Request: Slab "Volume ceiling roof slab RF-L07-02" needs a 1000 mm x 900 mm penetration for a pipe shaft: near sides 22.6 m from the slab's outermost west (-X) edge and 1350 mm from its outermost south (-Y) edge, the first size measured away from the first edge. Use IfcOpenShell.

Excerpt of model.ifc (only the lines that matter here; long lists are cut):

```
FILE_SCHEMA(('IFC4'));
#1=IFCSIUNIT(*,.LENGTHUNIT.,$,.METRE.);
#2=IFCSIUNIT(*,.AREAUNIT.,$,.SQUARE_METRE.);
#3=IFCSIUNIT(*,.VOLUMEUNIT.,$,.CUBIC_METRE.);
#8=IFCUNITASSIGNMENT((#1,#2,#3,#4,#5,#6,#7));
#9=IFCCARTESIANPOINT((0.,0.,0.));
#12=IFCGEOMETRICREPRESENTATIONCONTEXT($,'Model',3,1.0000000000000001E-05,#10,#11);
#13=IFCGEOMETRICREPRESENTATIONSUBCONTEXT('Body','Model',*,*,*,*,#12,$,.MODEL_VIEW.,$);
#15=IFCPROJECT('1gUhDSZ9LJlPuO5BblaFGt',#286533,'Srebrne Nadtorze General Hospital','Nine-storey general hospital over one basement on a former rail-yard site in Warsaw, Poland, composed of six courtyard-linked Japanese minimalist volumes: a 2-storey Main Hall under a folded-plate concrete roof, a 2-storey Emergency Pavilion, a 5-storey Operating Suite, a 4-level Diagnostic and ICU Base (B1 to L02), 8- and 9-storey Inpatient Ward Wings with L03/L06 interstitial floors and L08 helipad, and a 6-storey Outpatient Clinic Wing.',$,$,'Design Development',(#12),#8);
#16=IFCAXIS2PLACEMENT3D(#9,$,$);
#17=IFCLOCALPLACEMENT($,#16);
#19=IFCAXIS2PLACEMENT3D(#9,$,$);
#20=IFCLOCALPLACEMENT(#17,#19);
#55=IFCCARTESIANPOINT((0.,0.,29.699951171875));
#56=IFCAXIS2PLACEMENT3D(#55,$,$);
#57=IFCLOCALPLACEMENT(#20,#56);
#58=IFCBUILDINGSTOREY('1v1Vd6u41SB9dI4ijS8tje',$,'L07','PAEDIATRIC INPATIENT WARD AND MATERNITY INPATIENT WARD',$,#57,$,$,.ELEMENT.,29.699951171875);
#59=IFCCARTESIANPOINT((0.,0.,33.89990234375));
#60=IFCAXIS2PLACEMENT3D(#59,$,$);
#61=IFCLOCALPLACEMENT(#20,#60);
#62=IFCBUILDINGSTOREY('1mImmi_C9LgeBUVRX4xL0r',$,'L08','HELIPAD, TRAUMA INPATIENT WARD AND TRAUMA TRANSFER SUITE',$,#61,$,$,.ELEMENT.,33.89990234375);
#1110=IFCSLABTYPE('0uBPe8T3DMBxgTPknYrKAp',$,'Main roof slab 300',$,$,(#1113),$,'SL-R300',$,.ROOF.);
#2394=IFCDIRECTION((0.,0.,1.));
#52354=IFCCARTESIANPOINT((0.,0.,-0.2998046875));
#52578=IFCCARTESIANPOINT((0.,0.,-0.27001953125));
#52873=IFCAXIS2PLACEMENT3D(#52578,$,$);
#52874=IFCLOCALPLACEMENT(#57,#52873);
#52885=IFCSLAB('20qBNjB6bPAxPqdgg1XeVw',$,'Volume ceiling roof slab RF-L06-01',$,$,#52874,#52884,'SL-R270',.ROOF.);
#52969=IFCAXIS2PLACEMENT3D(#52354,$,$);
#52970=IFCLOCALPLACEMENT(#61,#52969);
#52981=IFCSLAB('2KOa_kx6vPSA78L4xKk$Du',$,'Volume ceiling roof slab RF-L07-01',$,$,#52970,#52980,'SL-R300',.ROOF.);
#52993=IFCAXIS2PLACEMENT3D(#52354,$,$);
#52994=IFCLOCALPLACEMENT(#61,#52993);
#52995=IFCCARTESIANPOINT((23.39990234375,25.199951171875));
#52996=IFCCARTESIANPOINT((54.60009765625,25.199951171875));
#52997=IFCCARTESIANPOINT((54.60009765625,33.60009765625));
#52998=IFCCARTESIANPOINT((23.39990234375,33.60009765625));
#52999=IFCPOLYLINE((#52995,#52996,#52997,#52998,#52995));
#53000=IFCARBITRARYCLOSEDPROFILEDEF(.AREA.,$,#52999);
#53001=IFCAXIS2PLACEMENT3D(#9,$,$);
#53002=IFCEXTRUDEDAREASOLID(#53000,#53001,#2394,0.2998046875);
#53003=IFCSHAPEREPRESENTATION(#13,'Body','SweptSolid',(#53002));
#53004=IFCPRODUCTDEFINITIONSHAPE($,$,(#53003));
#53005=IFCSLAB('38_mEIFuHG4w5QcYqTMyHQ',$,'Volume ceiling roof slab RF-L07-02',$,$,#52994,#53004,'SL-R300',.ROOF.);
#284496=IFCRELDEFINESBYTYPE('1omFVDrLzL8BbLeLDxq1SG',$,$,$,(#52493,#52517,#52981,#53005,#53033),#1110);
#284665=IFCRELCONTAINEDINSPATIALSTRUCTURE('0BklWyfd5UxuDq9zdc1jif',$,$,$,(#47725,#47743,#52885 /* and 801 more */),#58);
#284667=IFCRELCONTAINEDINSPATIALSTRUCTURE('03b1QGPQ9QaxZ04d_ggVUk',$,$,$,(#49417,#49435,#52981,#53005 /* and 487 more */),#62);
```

```python
import numpy as np
import ifcopenshell
import ifcopenshell.api.feature
import ifcopenshell.api.geometry
import ifcopenshell.api.root
import ifcopenshell.geom
import ifcopenshell.util.placement
import ifcopenshell.util.representation
import ifcopenshell.util.shape
import ifcopenshell.util.unit

model = ifcopenshell.open("model.ifc")
unit_scale = ifcopenshell.util.unit.calculate_unit_scale(model)
settings = ifcopenshell.geom.settings()


def volume(element):
    """Net volume in cubic metres, openings subtracted."""
    shape = ifcopenshell.geom.create_shape(settings, element)
    return ifcopenshell.util.shape.get_volume(shape.geometry)


slab = model.by_guid("38_mEIFuHG4w5QcYqTMyHQ")
before = volume(slab)

# Extent in the slab's own axes, in metres. The edges named are its -X and -Y sides.
slab_shape = ifcopenshell.geom.create_shape(settings, slab)
vertices = ifcopenshell.util.shape.get_vertices(slab_shape.geometry)
x_min, y_min, bottom = vertices.min(axis=0)
top = vertices[:, 2].max()

opening = ifcopenshell.api.root.create_entity(model, ifc_class="IfcOpeningElement", name="Pipe shaft opening", predefined_type="OPENING")
context = ifcopenshell.util.representation.get_context(model, "Model", "Body", "MODEL_VIEW")
width, depth = 1, 0.9
outline = [(0.0, 0.0), (width, 0.0), (width, depth), (0.0, depth), (0.0, 0.0)]
# Overshoot both faces by 50 mm so the cut is clean.
shape = ifcopenshell.api.geometry.add_slab_representation(
    model, context=context, depth=top - bottom + 0.1, polyline=outline
)
ifcopenshell.api.geometry.assign_representation(model, product=opening, representation=shape)

matrix = ifcopenshell.util.placement.get_local_placement(slab.ObjectPlacement)
matrix[:, 3] = matrix @ np.append(np.array([x_min + 22.6, y_min + 1.35, bottom - 0.05]) / unit_scale, 1.0)
ifcopenshell.api.geometry.edit_object_placement(model, product=opening, matrix=matrix, is_si=False)
ifcopenshell.api.feature.add_feature(model, feature=opening, element=slab)

after = volume(slab)

print(f"slab volume {before:.3f} -> {after:.3f} m3")

model.write("model_edited.ifc")
```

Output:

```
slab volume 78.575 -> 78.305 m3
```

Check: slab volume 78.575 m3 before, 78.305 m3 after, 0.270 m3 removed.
